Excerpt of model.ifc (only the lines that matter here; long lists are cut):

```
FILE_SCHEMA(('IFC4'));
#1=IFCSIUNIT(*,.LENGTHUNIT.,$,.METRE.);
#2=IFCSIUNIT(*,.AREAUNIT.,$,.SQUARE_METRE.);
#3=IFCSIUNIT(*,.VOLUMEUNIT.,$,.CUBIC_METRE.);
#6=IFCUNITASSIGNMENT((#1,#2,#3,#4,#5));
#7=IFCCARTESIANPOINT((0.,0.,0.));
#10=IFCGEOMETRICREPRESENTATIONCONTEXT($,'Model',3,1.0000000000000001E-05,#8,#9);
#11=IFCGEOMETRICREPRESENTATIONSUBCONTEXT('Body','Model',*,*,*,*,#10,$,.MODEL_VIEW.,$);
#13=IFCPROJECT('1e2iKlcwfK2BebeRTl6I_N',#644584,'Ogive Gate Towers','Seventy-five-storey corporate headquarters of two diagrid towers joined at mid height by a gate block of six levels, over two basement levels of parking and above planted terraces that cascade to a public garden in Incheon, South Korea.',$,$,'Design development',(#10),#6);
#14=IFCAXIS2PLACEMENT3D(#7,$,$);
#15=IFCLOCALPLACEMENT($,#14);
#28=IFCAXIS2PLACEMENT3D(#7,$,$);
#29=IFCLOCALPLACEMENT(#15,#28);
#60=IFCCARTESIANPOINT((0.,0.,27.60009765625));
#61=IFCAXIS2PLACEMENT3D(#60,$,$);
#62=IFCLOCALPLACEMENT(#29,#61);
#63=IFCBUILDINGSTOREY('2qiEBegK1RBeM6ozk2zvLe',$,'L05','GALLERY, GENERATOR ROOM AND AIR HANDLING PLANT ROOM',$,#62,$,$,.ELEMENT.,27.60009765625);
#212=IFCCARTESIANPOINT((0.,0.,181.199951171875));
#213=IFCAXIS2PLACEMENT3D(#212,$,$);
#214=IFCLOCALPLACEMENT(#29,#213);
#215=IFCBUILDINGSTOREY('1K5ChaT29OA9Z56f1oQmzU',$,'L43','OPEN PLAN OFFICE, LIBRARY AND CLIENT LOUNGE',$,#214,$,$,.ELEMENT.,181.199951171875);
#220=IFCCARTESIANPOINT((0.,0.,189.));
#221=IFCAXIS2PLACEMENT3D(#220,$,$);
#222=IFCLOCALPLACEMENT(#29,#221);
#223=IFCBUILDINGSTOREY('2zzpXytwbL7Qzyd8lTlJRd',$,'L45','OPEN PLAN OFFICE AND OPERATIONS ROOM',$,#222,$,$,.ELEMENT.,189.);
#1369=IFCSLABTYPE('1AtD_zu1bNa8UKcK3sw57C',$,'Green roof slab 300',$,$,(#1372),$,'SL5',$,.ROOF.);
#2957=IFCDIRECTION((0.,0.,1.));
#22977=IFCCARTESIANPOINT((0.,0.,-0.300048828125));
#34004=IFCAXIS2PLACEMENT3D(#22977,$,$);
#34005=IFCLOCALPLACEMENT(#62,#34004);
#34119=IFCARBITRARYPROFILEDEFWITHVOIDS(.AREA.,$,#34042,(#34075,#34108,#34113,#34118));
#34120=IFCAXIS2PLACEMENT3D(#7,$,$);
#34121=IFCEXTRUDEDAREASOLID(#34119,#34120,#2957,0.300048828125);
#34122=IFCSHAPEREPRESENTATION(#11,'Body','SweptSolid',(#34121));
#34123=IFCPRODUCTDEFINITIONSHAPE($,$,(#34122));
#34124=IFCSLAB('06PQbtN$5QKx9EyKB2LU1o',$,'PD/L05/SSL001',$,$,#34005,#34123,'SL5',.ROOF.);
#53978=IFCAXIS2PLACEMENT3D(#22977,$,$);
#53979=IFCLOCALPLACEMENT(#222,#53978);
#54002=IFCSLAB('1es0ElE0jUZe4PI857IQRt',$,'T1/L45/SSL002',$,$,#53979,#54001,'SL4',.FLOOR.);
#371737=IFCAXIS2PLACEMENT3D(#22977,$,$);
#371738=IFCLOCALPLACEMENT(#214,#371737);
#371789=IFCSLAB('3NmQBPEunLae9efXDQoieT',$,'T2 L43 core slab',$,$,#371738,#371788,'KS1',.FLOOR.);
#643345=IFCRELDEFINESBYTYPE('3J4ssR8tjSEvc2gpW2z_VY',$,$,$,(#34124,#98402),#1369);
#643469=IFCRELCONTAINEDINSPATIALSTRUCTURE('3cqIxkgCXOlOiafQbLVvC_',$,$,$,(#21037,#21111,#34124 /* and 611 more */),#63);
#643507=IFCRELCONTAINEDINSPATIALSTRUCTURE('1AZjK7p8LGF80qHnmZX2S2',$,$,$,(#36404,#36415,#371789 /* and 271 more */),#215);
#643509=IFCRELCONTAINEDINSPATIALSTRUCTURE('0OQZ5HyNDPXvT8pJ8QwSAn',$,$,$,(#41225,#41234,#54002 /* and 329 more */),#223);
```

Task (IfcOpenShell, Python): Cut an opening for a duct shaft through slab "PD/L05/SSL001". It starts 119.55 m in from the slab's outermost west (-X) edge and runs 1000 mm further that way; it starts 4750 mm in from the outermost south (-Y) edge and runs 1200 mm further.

```python
import numpy as np
import ifcopenshell
import ifcopenshell.api.feature
import ifcopenshell.api.geometry
import ifcopenshell.api.root
import ifcopenshell.geom
import ifcopenshell.util.placement
import ifcopenshell.util.representation
import ifcopenshell.util.shape
import ifcopenshell.util.unit

model = ifcopenshell.open("model.ifc")
unit_scale = ifcopenshell.util.unit.calculate_unit_scale(model)
settings = ifcopenshell.geom.settings()


def volume(element):
    """Net volume in cubic metres, openings subtracted."""
    shape = ifcopenshell.geom.create_shape(settings, element)
    return ifcopenshell.util.shape.get_volume(shape.geometry)


slab = model.by_guid("06PQbtN$5QKx9EyKB2LU1o")
before = volume(slab)

# Extent in the slab's own axes, in metres. The edges named are its -X and -Y sides.
slab_shape = ifcopenshell.geom.create_shape(settings, slab)
vertices = ifcopenshell.util.shape.get_vertices(slab_shape.geometry)
x_min, y_min, bottom = vertices.min(axis=0)
top = vertices[:, 2].max()

opening = ifcopenshell.api.root.create_entity(model, ifc_class="IfcOpeningElement", name="Duct shaft opening", predefined_type="OPENING")
context = ifcopenshell.util.representation.get_context(model, "Model", "Body", "MODEL_VIEW")
width, depth = 1, 1.2
outline = [(0.0, 0.0), (width, 0.0), (width, depth), (0.0, depth), (0.0, 0.0)]
# Overshoot both faces by 50 mm so the cut is clean.
shape = ifcopenshell.api.geometry.add_slab_representation(
    model, context=context, depth=top - bottom + 0.1, polyline=outline
)
ifcopenshell.api.geometry.assign_representation(model, product=opening, representation=shape)

matrix = ifcopenshell.util.placement.get_local_placement(slab.ObjectPlacement)
matrix[:, 3] = matrix @ np.append(np.array([x_min + 119.55, y_min + 4.75, bottom - 0.05]) / unit_scale, 1.0)
ifcopenshell.api.geometry.edit_object_placement(model, product=opening, matrix=matrix, is_si=False)
ifcopenshell.api.feature.add_feature(model, feature=opening, element=slab)

after = volume(slab)

print(f"slab volume {before:.3f} -> {after:.3f} m3")

model.write("model_edited.ifc")
```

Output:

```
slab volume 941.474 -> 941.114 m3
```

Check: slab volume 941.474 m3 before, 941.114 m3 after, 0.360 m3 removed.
